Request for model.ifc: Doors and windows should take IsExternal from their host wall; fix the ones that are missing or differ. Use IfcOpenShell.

First a look at what the model holds.

```python
import ifcopenshell
import ifcopenshell.util.element

model = ifcopenshell.open("model.ifc")
print(model.schema)
seen = {}
for e in model.by_type("IfcDoor") + model.by_type("IfcWindow"):
    if not e.FillsVoids:
        continue
    host = e.FillsVoids[0].RelatingOpeningElement.VoidsElements[0].RelatingBuildingElement
    own = ifcopenshell.util.element.get_pset(e, f"Pset_{e.is_a()[3:].removesuffix('StandardCase')}Common", "IsExternal")
    wall = ifcopenshell.util.element.get_pset(host, "Pset_WallCommon", "IsExternal")
    seen[e.is_a(), own, wall] = seen.get((e.is_a(), own, wall), 0) + 1
for (cls, own, wall), count in sorted(seen.items(), key=str):
    print(count, cls, "IsExternal:", own, "| host wall:", wall)
```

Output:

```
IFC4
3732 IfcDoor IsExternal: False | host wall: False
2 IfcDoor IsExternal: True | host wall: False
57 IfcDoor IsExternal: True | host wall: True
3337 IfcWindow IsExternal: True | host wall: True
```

```python
import ifcopenshell
import ifcopenshell.api.pset
import ifcopenshell.util.element

model = ifcopenshell.open("model.ifc")

count = 0
for ifc_class, pset_name in (("IfcDoor", "Pset_DoorCommon"), ("IfcWindow", "Pset_WindowCommon")):
    for e in model.by_type(ifc_class):
        if not e.FillsVoids:
            continue
        host = e.FillsVoids[0].RelatingOpeningElement.VoidsElements[0].RelatingBuildingElement
        external = ifcopenshell.util.element.get_pset(host, "Pset_WallCommon", "IsExternal")
        if external is None or ifcopenshell.util.element.get_pset(e, pset_name, "IsExternal") == external:
            continue
        pset = ifcopenshell.api.pset.add_pset(model, product=e, name=pset_name)
        ifcopenshell.api.pset.edit_pset(model, pset=pset, properties={"IsExternal": external})
        count += 1

print(count, "updated")

model.write("model_v2.ifc")
```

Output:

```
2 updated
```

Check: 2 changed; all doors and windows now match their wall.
